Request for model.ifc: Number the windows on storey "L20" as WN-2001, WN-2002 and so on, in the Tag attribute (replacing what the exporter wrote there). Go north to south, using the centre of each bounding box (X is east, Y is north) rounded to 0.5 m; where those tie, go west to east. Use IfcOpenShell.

First a look at what the model holds.

```python
import ifcopenshell
import ifcopenshell.util.element
import ifcopenshell.util.placement

model = ifcopenshell.open("model.ifc")
print(model.schema)
storey = next(s for s in model.by_type("IfcBuildingStorey") if s.Name == "L20")
windows = [e for e in ifcopenshell.util.element.get_decomposition(storey) if e.is_a("IfcWindow")]
for e in sorted(windows, key=lambda e: e.id()):
    origin = ifcopenshell.util.placement.get_local_placement(e.ObjectPlacement)[:3, 3]
    print(e.id(), e.Tag, e.Name, origin.round(2) + 0.0, sep=" | ")
```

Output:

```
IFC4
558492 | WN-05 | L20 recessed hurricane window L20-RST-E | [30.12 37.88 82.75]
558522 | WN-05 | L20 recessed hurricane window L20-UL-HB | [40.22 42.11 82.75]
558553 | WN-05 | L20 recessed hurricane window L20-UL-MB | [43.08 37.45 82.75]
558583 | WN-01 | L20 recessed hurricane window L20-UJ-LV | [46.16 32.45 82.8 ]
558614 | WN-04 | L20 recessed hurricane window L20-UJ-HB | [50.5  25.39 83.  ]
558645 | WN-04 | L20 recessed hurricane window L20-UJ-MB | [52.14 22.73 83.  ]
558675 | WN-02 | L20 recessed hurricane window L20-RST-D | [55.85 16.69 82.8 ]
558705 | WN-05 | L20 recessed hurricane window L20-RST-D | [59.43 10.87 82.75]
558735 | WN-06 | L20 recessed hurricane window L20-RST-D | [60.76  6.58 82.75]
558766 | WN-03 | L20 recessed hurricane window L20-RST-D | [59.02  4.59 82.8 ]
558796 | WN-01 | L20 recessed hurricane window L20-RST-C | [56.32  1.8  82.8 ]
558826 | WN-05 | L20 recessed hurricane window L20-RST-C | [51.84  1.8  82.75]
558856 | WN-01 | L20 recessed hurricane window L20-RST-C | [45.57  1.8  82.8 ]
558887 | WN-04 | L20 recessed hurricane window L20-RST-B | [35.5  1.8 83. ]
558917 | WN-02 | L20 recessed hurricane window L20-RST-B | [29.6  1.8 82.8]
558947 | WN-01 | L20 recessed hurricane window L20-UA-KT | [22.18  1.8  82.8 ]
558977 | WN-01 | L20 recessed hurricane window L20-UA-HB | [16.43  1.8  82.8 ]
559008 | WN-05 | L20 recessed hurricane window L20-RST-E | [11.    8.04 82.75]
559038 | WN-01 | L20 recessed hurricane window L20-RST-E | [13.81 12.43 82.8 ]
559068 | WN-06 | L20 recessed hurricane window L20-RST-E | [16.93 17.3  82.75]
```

```python
import ifcopenshell
import ifcopenshell.geom
import ifcopenshell.util.element
import ifcopenshell.util.shape

model = ifcopenshell.open("model.ifc")
settings = ifcopenshell.geom.settings()
settings.set("use-world-coords", True)


def centre(element):
    shape = ifcopenshell.geom.create_shape(settings, element)
    return ifcopenshell.util.shape.get_bbox_centroid(shape.geometry)


storey = next(s for s in model.by_type("IfcBuildingStorey") if s.Name == "L20")
windows = [e for e in ifcopenshell.util.element.get_decomposition(storey) if e.is_a("IfcWindow")]

# Insertion points can sit at a corner or the storey origin, so sort by the geometry (in metres).
centres = {e: centre(e) for e in windows}
windows.sort(key=lambda e: (-round(centres[e][1] / 0.5), centres[e][0]))

for i, e in enumerate(windows, start=1):
    number = f"WN-20{i:02d}"
    e.Tag = number
    print(e.id(), number)

model.write("model-out.ifc")
```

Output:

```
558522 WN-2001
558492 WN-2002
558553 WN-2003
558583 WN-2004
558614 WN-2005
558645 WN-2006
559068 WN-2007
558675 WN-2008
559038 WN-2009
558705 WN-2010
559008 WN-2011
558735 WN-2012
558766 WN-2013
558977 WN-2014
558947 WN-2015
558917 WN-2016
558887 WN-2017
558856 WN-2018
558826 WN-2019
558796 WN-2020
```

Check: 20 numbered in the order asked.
